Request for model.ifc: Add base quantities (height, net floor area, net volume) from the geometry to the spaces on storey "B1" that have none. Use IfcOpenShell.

First a look at what the model holds.

```python
import ifcopenshell
import ifcopenshell.util.element
import ifcopenshell.util.unit

model = ifcopenshell.open("model.ifc")
print(model.schema)
for unit_type in ("LENGTHUNIT", "AREAUNIT", "VOLUMEUNIT"):
    print(unit_type, ifcopenshell.util.unit.calculate_unit_scale(model, unit_type))
storey = next(s for s in model.by_type("IfcBuildingStorey") if s.Name == "B1")
spaces = [e for e in ifcopenshell.util.element.get_decomposition(storey) if e.is_a("IfcSpace")]
for e in sorted(spaces, key=lambda e: e.id()):
    print(e.id(), e.is_a(), e.Name, list(ifcopenshell.util.element.get_psets(e, qtos_only=True)), sep=" | ")
```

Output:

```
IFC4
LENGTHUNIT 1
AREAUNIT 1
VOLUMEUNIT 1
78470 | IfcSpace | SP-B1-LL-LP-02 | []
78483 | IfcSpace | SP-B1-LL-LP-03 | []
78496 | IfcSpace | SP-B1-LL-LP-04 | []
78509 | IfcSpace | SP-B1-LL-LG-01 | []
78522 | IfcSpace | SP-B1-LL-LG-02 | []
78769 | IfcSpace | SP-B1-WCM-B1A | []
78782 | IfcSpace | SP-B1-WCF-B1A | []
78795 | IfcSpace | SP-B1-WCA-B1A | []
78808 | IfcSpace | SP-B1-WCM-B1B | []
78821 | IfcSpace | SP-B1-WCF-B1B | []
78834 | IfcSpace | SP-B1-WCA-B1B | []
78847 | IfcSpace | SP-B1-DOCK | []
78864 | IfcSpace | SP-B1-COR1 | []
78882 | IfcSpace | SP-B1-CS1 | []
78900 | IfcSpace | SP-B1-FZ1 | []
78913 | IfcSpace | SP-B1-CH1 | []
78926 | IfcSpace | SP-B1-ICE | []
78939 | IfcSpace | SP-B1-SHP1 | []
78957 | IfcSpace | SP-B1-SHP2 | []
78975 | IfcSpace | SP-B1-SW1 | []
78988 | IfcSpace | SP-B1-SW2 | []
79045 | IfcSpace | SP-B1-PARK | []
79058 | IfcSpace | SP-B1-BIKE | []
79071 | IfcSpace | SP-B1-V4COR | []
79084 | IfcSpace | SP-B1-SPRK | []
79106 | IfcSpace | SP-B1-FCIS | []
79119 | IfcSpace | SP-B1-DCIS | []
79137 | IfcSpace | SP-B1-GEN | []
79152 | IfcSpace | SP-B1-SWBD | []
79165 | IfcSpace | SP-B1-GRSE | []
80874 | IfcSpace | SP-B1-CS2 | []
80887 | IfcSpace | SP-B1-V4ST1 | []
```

```python
import ifcopenshell
import ifcopenshell.api.pset
import ifcopenshell.geom
import ifcopenshell.util.element
import ifcopenshell.util.shape
import ifcopenshell.util.unit

model = ifcopenshell.open("model.ifc")
unit_scale = ifcopenshell.util.unit.calculate_unit_scale(model)
area_scale = ifcopenshell.util.unit.calculate_unit_scale(model, "AREAUNIT")
volume_scale = ifcopenshell.util.unit.calculate_unit_scale(model, "VOLUMEUNIT")
settings = ifcopenshell.geom.settings()

storey = next(s for s in model.by_type("IfcBuildingStorey") if s.Name == "B1")
spaces = [e for e in ifcopenshell.util.element.get_decomposition(storey) if e.is_a("IfcSpace")]

for e in sorted(spaces, key=lambda e: e.id()):
    if ifcopenshell.util.element.get_psets(e, qtos_only=True, should_inherit=False):
        continue
    # Geometry comes back in metres, in the element's own axes.
    shape = ifcopenshell.geom.create_shape(settings, e)
    values = {
        "Height": ifcopenshell.util.shape.get_z(shape.geometry) / unit_scale,
        "NetFloorArea": ifcopenshell.util.shape.get_footprint_area(shape.geometry) / area_scale,
        "NetVolume": ifcopenshell.util.shape.get_volume(shape.geometry) / volume_scale,
    }
    qto = ifcopenshell.api.pset.add_qto(model, product=e, name="Qto_SpaceBaseQuantities")
    ifcopenshell.api.pset.edit_qto(model, qto=qto, properties=values)
    print(e.id(), {k: round(v, 3) for k, v in values.items()})

model.write("model_v2.ifc")
```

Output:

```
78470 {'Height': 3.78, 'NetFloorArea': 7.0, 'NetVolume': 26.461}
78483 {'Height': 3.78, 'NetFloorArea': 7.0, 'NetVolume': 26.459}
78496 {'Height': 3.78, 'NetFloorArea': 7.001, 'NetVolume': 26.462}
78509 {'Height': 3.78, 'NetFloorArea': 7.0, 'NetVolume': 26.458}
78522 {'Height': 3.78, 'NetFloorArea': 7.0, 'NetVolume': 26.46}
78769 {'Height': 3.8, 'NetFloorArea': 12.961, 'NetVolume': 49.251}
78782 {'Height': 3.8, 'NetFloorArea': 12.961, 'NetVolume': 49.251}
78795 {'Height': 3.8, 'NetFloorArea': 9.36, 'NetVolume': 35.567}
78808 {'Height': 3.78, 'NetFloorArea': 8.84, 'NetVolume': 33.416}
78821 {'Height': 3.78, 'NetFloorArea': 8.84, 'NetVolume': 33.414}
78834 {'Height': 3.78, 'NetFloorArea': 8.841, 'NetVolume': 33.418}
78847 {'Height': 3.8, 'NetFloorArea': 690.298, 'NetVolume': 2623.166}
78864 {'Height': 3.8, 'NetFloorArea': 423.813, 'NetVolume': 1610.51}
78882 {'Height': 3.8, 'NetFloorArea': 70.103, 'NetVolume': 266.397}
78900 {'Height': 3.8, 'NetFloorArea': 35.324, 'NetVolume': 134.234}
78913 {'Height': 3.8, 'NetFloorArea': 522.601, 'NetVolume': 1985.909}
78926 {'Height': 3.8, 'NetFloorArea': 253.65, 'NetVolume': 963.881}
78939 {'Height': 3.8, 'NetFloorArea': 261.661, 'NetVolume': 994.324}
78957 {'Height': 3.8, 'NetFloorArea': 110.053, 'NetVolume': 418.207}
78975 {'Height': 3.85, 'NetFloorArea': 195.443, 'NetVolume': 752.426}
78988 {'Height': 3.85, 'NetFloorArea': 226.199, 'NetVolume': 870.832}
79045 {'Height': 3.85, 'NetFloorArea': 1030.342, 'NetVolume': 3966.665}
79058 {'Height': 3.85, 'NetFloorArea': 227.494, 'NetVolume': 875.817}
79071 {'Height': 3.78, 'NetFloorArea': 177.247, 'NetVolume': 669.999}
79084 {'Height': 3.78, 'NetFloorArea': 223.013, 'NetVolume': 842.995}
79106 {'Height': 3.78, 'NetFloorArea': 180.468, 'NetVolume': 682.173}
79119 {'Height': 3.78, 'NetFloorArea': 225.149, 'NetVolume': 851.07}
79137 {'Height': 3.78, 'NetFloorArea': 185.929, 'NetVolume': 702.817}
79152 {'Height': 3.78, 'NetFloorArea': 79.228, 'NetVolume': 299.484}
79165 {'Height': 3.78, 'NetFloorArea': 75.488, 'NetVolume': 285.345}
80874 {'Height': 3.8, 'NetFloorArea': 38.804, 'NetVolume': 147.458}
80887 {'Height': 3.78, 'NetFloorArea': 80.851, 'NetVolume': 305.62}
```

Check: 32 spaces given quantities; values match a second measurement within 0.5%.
